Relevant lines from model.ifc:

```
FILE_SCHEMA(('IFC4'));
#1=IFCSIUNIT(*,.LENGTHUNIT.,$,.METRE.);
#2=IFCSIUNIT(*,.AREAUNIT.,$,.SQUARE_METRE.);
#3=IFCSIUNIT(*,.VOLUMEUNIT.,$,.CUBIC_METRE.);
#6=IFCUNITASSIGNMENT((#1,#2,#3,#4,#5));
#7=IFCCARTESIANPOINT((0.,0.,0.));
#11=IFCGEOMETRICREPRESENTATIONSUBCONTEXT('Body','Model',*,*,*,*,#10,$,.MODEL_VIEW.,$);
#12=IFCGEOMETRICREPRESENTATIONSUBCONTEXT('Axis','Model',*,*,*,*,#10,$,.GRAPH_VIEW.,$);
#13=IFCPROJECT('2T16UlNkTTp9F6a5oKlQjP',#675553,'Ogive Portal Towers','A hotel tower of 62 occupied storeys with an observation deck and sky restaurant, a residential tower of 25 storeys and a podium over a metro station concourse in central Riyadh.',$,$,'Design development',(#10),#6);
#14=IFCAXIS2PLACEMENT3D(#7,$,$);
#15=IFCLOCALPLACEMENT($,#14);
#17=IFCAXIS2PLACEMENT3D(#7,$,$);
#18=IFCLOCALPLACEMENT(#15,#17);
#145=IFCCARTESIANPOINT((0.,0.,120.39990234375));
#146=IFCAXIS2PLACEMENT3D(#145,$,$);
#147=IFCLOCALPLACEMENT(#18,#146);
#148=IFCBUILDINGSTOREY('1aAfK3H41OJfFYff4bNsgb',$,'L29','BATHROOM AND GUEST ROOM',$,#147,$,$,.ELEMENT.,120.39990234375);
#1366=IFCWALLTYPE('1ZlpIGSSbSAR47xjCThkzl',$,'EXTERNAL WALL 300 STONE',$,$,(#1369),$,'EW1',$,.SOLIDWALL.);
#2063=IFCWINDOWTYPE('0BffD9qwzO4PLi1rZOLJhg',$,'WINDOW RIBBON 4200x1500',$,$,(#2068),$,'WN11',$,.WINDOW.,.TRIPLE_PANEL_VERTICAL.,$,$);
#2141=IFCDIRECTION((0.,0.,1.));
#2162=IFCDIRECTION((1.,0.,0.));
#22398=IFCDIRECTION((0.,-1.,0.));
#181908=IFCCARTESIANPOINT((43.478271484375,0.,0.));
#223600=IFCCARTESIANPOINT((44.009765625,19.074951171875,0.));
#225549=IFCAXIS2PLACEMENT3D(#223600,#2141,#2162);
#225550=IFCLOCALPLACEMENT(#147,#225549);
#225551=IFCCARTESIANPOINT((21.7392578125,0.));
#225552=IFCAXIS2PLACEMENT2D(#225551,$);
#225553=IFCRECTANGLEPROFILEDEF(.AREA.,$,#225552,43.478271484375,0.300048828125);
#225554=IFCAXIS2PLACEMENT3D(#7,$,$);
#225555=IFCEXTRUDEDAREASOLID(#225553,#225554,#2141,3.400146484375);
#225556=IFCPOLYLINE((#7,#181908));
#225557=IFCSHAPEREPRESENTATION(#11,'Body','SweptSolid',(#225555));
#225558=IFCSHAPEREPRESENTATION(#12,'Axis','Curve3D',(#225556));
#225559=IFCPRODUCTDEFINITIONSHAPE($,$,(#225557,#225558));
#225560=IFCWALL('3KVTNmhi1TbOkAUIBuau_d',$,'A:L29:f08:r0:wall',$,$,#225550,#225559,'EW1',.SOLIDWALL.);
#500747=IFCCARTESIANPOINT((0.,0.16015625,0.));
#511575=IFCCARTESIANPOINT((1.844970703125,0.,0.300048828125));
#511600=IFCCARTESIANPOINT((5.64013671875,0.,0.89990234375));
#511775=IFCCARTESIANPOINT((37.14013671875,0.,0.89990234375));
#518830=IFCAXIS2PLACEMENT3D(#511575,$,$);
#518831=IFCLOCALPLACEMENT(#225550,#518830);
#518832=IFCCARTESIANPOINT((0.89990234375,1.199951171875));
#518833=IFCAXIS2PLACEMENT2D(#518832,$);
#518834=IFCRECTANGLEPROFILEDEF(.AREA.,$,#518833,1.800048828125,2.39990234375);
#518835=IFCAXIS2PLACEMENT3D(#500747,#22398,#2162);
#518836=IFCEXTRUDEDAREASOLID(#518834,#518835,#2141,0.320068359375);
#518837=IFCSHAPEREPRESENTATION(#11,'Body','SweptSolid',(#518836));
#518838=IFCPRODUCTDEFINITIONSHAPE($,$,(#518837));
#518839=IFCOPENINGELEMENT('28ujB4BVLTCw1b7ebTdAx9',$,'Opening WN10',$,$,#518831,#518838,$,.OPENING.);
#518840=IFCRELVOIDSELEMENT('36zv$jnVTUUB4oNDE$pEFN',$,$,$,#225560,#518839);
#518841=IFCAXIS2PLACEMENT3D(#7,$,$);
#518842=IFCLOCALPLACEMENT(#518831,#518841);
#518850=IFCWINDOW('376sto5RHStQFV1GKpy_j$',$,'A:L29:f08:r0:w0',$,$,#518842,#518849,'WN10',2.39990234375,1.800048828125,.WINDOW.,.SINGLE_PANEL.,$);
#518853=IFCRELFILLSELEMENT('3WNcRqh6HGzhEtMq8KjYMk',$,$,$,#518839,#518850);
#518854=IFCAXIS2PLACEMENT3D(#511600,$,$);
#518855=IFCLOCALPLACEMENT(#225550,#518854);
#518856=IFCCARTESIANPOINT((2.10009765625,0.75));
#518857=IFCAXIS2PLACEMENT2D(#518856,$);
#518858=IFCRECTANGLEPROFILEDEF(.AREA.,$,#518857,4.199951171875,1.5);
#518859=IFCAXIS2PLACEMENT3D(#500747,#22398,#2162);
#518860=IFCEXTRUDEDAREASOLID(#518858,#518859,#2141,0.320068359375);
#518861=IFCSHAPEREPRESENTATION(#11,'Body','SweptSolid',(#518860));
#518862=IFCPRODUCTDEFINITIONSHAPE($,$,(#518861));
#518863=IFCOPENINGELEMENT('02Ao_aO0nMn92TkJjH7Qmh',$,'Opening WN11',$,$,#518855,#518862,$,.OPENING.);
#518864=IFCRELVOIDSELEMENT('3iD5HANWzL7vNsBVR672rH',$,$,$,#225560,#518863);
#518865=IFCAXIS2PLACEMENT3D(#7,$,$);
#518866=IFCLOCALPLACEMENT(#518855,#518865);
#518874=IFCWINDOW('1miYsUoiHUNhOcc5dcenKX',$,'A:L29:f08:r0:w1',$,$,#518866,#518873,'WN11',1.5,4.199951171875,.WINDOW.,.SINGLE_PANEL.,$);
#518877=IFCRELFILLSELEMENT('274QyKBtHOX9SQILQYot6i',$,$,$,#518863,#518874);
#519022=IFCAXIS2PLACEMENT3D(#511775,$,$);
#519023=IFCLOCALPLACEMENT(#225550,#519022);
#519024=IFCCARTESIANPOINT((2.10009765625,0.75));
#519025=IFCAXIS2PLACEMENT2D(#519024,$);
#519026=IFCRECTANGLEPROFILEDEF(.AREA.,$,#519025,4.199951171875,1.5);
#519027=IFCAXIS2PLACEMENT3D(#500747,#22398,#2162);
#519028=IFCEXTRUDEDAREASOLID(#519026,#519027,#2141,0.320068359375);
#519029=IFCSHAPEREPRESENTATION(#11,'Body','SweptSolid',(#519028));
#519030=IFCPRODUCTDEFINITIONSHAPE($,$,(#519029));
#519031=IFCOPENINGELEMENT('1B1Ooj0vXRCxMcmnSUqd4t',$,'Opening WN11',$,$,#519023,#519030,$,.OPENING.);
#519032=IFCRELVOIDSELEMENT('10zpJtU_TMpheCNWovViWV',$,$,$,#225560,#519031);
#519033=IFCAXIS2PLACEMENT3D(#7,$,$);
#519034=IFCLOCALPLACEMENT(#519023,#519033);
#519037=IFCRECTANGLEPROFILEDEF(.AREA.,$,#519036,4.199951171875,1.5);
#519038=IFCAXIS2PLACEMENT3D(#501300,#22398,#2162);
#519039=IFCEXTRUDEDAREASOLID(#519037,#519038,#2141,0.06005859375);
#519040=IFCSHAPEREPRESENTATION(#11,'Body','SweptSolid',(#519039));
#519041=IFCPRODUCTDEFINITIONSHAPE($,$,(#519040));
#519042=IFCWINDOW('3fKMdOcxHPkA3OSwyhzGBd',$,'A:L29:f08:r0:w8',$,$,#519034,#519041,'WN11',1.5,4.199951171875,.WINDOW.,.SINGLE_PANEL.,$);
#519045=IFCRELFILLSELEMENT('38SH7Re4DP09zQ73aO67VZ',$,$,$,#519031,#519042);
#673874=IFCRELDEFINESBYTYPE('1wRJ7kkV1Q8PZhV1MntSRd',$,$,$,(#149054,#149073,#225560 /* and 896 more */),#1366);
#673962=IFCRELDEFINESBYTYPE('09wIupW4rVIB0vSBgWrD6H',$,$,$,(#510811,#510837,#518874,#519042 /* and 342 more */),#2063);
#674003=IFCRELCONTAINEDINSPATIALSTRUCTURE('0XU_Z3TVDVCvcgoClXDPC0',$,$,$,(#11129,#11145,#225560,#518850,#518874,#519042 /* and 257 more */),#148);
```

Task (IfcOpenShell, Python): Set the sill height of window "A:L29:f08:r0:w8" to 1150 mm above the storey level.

```python
import numpy as np
import ifcopenshell
import ifcopenshell.api.geometry
import ifcopenshell.geom
import ifcopenshell.util.element
import ifcopenshell.util.placement
import ifcopenshell.util.shape
import ifcopenshell.util.unit

model = ifcopenshell.open("model.ifc")
unit_scale = ifcopenshell.util.unit.calculate_unit_scale(model)

window = model.by_id(519042)
opening = window.FillsVoids[0].RelatingOpeningElement
storey = ifcopenshell.util.element.get_container(window, ifc_class="IfcBuildingStorey")
level = ifcopenshell.util.placement.get_local_placement(storey.ObjectPlacement)[2, 3]

# The opening's origin need not be at the sill, so measure its lowest point.
shape = ifcopenshell.geom.create_shape(ifcopenshell.geom.settings(), opening)
bottom = ifcopenshell.util.shape.get_shape_bottom_elevation(shape, shape.geometry) / unit_scale
dz = level + 1.15 / unit_scale - bottom

shift = np.array([0.0, 0.0, dz])
# The window is placed relative to its opening, so it follows when the opening moves.
matrix = ifcopenshell.util.placement.get_local_placement(opening.ObjectPlacement)
matrix[:3, 3] += shift
ifcopenshell.api.geometry.edit_object_placement(
    model, product=opening, matrix=matrix, is_si=False, should_transform_children=True
)

print(f"moved by {dz * unit_scale:+.3f} m")

model.write("model_edited.ifc")
```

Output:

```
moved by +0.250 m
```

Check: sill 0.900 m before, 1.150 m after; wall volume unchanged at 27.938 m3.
